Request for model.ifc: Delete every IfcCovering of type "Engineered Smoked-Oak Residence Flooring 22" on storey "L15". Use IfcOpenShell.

First a look at what the model holds.

```python
import ifcopenshell
import ifcopenshell.util.element

model = ifcopenshell.open("model.ifc")
print(model.schema)
storey = next(s for s in model.by_type("IfcBuildingStorey") if s.Name == "L15")
coverings = [e for e in ifcopenshell.util.element.get_decomposition(storey) if e.is_a("IfcCovering")]
seen = {}
for e in coverings:
    element_type = ifcopenshell.util.element.get_type(e)
    name = element_type.Name if element_type not in (None, e) else None
    seen[name] = seen.get(name, 0) + 1
for name, count in sorted(seen.items(), key=str):
    print(count, "x", name)
```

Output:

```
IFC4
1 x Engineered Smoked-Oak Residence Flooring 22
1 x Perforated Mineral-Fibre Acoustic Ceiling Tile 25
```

```python
import ifcopenshell
import ifcopenshell.api.root
import ifcopenshell.util.element

model = ifcopenshell.open("model.ifc")

storey = next(s for s in model.by_type("IfcBuildingStorey") if s.Name == "L15")
coverings = [e for e in ifcopenshell.util.element.get_decomposition(storey) if e.is_a("IfcCovering")]
targets = [e for e in coverings if (t := ifcopenshell.util.element.get_type(e)) not in (None, e) and t.Name == "Engineered Smoked-Oak Residence Flooring 22"]

for e in targets:
    ifcopenshell.api.root.remove_product(model, product=e)
print(len(targets), "removed")

model.write("model-out.ifc")
```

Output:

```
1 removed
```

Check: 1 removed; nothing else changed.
